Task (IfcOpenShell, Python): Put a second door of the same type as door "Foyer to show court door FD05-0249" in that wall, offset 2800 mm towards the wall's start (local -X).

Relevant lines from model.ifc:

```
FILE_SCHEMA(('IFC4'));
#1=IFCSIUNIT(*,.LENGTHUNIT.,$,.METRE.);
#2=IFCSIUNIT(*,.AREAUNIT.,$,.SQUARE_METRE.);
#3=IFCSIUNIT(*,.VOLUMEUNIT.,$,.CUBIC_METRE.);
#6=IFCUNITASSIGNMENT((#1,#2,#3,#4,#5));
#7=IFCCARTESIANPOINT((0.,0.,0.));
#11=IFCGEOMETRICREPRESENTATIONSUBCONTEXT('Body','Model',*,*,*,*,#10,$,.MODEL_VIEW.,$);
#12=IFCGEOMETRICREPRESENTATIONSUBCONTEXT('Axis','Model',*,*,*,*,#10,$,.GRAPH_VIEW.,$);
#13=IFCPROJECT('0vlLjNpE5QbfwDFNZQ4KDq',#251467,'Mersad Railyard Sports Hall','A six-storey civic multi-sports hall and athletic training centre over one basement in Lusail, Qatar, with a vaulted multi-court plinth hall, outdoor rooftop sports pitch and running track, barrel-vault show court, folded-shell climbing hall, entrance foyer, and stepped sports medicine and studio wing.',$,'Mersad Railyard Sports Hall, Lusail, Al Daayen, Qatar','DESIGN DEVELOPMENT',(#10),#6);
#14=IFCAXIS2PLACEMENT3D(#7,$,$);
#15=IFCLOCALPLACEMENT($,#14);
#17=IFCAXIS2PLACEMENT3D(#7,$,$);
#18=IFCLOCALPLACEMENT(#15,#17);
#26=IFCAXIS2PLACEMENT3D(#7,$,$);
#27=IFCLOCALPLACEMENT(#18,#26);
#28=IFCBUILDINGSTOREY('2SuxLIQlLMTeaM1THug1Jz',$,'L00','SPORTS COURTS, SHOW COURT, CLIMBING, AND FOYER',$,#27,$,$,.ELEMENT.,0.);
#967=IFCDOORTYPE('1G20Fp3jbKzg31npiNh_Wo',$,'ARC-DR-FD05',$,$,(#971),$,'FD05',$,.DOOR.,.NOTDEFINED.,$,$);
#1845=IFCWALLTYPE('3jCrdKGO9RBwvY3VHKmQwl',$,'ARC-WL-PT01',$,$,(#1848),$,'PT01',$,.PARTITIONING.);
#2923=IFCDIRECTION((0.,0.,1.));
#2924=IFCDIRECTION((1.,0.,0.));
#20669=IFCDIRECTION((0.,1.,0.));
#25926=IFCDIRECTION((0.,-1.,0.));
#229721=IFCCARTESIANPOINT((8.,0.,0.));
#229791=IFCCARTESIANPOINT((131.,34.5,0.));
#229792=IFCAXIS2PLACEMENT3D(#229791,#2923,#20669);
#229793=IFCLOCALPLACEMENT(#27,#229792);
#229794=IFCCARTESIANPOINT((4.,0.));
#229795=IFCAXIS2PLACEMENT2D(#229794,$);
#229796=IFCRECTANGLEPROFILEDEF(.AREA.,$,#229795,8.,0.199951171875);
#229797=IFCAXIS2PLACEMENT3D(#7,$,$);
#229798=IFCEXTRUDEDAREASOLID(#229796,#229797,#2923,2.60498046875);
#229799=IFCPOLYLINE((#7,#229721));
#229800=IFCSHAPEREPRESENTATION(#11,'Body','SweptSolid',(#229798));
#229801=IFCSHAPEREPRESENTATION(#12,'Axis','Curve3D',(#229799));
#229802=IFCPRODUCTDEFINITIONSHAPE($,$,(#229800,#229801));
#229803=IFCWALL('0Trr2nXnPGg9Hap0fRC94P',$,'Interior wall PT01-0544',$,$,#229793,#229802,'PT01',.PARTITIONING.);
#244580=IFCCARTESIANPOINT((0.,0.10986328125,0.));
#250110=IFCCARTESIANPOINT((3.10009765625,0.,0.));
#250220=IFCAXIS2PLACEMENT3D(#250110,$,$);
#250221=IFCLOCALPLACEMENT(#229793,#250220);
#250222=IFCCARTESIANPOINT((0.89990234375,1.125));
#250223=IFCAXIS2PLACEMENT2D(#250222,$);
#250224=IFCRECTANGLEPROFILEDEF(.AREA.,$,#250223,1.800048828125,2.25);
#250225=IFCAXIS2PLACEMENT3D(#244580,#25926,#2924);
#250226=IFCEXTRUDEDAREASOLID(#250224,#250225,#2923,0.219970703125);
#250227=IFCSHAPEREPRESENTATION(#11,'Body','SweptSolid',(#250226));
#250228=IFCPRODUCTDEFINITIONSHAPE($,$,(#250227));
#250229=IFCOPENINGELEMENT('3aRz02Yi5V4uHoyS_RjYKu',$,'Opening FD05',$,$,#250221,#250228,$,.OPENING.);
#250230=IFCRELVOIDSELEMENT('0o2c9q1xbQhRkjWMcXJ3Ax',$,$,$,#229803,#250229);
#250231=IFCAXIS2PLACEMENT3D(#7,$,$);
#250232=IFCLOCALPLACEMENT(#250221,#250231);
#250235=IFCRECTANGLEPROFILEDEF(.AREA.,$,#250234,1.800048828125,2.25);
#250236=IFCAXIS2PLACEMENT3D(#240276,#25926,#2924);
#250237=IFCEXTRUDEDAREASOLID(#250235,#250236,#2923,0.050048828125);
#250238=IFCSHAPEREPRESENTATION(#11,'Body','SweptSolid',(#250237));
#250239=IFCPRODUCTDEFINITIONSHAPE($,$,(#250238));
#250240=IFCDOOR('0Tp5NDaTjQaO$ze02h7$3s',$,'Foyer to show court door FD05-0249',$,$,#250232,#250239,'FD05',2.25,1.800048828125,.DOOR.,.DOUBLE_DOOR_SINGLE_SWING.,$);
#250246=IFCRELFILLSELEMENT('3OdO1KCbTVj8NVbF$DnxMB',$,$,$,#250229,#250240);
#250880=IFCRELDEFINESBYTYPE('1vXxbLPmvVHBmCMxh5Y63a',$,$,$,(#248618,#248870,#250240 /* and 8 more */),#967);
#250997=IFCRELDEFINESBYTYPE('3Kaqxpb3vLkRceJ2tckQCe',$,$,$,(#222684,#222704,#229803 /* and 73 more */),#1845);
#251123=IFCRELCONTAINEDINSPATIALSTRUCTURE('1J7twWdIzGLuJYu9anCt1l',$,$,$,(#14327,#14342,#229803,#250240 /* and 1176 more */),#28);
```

```python
import ifcopenshell
import ifcopenshell.api.feature
import ifcopenshell.api.geometry
import ifcopenshell.api.root
import ifcopenshell.geom
import ifcopenshell.util.element
import ifcopenshell.util.placement
import ifcopenshell.util.shape

model = ifcopenshell.open("model.ifc")
settings = ifcopenshell.geom.settings()


def volume(element):
    """Net volume in cubic metres, openings subtracted."""
    shape = ifcopenshell.geom.create_shape(settings, element)
    return ifcopenshell.util.shape.get_volume(shape.geometry)


door = model.by_guid("0Tp5NDaTjQaO$ze02h7$3s")
opening = door.FillsVoids[0].RelatingOpeningElement
wall = opening.VoidsElements[0].RelatingBuildingElement
before = volume(wall)
shift = ifcopenshell.util.placement.get_local_placement(wall.ObjectPlacement)[:3, 0] * -2.8

# copy_class copies the void relationship, type, container and properties, but no geometry.
new_opening = ifcopenshell.api.root.copy_class(model, product=opening)
new_opening.Representation = ifcopenshell.util.element.copy_deep(
    model, opening.Representation, exclude=["IfcGeometricRepresentationContext", "IfcRepresentationMap"]
)
new_door = ifcopenshell.api.root.copy_class(model, product=door)
new_door.Representation = ifcopenshell.util.element.copy_deep(
    model, door.Representation, exclude=["IfcGeometricRepresentationContext", "IfcRepresentationMap"]
)
new_door.Tag = None
ifcopenshell.api.feature.add_filling(model, opening=new_opening, element=new_door)

for old, new in ((opening, new_opening), (door, new_door)):
    matrix = ifcopenshell.util.placement.get_local_placement(old.ObjectPlacement)
    matrix[:3, 3] += shift
    ifcopenshell.api.geometry.edit_object_placement(model, product=new, matrix=matrix, is_si=False)

after = volume(wall)

print(f"wall volume {before:.3f} -> {after:.3f} m3")

model.write("model-out.ifc")
```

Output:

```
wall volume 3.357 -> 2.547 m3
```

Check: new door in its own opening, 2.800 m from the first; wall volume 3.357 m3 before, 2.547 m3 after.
